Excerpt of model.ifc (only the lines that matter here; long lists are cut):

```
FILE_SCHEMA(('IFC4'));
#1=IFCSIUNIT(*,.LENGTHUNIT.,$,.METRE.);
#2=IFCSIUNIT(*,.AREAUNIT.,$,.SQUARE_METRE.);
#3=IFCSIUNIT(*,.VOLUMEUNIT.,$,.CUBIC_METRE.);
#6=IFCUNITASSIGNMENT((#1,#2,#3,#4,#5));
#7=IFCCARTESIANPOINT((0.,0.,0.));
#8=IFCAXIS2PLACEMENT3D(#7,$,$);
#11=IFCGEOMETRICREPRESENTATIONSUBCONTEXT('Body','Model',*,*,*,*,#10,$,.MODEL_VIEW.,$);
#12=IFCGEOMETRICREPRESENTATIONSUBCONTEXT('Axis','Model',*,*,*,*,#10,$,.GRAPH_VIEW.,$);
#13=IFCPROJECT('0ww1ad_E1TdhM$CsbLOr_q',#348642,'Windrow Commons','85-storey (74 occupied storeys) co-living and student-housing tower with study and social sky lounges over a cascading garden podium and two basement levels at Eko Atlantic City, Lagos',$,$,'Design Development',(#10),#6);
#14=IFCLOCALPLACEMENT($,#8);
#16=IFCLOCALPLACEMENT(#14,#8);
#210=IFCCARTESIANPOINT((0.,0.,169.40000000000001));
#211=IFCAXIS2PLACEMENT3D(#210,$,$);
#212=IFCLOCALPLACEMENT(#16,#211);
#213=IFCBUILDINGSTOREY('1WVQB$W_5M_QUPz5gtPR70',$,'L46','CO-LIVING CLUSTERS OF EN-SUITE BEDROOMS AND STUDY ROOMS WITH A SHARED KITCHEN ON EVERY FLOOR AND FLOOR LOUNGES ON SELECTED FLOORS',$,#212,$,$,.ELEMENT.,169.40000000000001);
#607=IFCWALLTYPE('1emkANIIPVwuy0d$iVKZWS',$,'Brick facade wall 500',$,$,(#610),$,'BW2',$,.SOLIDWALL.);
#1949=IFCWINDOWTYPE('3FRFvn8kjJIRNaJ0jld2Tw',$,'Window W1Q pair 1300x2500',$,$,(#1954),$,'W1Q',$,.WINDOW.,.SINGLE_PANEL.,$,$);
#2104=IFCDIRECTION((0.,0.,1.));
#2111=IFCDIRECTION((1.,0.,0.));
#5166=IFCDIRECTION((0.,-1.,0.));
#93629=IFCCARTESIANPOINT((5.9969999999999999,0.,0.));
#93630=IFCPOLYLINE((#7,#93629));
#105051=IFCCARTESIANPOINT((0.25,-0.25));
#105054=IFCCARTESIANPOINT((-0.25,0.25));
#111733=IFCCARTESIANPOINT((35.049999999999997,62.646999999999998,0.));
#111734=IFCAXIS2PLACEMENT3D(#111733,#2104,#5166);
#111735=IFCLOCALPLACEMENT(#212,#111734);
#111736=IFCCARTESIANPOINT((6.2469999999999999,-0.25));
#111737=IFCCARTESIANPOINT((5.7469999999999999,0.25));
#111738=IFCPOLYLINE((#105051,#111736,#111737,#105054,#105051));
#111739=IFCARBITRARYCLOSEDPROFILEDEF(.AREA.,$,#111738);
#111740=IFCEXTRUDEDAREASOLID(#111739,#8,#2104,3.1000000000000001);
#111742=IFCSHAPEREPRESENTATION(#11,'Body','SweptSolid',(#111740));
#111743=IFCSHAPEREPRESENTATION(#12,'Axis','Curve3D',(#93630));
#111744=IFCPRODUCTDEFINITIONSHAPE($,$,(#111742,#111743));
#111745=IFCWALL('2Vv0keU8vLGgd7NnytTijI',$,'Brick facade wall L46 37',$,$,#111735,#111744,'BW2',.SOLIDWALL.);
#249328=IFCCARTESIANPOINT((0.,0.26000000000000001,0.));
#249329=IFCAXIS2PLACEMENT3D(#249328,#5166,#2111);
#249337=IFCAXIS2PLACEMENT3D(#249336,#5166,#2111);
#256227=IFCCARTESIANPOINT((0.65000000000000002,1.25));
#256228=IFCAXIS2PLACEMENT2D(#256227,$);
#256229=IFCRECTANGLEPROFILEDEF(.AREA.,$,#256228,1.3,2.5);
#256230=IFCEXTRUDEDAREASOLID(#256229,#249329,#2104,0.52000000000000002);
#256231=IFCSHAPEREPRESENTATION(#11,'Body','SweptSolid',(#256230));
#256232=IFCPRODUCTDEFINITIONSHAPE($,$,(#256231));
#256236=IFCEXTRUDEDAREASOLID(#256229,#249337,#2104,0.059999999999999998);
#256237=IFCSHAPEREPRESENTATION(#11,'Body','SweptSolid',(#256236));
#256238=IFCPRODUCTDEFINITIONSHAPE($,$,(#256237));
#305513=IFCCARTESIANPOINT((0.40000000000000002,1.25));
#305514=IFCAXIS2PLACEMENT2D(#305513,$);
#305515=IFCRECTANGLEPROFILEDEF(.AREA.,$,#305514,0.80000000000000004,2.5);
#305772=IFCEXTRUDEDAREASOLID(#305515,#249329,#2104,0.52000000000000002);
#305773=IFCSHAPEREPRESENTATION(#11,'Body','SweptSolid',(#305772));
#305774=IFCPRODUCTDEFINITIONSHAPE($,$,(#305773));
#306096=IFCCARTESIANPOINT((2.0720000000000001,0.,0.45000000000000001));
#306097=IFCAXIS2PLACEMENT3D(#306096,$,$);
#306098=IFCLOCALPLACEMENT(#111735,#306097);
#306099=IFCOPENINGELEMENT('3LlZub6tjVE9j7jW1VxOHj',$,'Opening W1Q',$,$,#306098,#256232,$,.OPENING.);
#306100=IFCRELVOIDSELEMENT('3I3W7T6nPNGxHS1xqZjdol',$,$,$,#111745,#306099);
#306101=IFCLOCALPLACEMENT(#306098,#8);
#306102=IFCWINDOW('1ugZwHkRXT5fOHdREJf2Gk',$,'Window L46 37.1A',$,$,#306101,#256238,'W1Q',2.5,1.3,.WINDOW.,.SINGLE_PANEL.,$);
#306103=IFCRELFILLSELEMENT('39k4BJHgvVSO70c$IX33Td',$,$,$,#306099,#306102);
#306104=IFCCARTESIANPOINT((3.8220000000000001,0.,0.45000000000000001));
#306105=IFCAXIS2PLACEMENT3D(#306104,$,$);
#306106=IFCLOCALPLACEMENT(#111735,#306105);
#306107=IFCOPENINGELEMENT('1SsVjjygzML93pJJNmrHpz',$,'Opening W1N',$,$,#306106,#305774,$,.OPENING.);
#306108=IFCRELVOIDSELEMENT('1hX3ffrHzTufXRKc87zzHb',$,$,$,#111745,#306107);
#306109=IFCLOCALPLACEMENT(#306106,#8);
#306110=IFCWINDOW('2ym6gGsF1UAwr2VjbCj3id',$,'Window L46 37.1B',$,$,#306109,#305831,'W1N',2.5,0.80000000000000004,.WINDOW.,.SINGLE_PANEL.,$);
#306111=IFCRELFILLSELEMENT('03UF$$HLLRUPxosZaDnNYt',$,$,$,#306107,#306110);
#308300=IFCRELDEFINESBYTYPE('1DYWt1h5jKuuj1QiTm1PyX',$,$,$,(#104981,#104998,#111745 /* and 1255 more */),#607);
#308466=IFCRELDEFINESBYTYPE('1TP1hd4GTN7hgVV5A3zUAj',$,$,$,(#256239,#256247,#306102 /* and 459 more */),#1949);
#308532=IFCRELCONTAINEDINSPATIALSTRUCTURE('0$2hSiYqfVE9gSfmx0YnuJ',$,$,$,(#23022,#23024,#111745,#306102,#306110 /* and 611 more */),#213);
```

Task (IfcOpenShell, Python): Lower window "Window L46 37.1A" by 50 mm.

```python
import numpy as np
import ifcopenshell
import ifcopenshell.api.geometry
import ifcopenshell.util.placement
import ifcopenshell.util.unit

model = ifcopenshell.open("model.ifc")
unit_scale = ifcopenshell.util.unit.calculate_unit_scale(model)

window = model.by_guid("1ugZwHkRXT5fOHdREJf2Gk")
opening = window.FillsVoids[0].RelatingOpeningElement
dz = -0.05

shift = np.array([0.0, 0.0, dz])
# The window is placed relative to its opening, so it follows when the opening moves.
matrix = ifcopenshell.util.placement.get_local_placement(opening.ObjectPlacement)
matrix[:3, 3] += shift
ifcopenshell.api.geometry.edit_object_placement(
    model, product=opening, matrix=matrix, is_si=False, should_transform_children=True
)

print(f"moved by {dz * unit_scale:+.3f} m")

model.write("model_edited.ifc")
```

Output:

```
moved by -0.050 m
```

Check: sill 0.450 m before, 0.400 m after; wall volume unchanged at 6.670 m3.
